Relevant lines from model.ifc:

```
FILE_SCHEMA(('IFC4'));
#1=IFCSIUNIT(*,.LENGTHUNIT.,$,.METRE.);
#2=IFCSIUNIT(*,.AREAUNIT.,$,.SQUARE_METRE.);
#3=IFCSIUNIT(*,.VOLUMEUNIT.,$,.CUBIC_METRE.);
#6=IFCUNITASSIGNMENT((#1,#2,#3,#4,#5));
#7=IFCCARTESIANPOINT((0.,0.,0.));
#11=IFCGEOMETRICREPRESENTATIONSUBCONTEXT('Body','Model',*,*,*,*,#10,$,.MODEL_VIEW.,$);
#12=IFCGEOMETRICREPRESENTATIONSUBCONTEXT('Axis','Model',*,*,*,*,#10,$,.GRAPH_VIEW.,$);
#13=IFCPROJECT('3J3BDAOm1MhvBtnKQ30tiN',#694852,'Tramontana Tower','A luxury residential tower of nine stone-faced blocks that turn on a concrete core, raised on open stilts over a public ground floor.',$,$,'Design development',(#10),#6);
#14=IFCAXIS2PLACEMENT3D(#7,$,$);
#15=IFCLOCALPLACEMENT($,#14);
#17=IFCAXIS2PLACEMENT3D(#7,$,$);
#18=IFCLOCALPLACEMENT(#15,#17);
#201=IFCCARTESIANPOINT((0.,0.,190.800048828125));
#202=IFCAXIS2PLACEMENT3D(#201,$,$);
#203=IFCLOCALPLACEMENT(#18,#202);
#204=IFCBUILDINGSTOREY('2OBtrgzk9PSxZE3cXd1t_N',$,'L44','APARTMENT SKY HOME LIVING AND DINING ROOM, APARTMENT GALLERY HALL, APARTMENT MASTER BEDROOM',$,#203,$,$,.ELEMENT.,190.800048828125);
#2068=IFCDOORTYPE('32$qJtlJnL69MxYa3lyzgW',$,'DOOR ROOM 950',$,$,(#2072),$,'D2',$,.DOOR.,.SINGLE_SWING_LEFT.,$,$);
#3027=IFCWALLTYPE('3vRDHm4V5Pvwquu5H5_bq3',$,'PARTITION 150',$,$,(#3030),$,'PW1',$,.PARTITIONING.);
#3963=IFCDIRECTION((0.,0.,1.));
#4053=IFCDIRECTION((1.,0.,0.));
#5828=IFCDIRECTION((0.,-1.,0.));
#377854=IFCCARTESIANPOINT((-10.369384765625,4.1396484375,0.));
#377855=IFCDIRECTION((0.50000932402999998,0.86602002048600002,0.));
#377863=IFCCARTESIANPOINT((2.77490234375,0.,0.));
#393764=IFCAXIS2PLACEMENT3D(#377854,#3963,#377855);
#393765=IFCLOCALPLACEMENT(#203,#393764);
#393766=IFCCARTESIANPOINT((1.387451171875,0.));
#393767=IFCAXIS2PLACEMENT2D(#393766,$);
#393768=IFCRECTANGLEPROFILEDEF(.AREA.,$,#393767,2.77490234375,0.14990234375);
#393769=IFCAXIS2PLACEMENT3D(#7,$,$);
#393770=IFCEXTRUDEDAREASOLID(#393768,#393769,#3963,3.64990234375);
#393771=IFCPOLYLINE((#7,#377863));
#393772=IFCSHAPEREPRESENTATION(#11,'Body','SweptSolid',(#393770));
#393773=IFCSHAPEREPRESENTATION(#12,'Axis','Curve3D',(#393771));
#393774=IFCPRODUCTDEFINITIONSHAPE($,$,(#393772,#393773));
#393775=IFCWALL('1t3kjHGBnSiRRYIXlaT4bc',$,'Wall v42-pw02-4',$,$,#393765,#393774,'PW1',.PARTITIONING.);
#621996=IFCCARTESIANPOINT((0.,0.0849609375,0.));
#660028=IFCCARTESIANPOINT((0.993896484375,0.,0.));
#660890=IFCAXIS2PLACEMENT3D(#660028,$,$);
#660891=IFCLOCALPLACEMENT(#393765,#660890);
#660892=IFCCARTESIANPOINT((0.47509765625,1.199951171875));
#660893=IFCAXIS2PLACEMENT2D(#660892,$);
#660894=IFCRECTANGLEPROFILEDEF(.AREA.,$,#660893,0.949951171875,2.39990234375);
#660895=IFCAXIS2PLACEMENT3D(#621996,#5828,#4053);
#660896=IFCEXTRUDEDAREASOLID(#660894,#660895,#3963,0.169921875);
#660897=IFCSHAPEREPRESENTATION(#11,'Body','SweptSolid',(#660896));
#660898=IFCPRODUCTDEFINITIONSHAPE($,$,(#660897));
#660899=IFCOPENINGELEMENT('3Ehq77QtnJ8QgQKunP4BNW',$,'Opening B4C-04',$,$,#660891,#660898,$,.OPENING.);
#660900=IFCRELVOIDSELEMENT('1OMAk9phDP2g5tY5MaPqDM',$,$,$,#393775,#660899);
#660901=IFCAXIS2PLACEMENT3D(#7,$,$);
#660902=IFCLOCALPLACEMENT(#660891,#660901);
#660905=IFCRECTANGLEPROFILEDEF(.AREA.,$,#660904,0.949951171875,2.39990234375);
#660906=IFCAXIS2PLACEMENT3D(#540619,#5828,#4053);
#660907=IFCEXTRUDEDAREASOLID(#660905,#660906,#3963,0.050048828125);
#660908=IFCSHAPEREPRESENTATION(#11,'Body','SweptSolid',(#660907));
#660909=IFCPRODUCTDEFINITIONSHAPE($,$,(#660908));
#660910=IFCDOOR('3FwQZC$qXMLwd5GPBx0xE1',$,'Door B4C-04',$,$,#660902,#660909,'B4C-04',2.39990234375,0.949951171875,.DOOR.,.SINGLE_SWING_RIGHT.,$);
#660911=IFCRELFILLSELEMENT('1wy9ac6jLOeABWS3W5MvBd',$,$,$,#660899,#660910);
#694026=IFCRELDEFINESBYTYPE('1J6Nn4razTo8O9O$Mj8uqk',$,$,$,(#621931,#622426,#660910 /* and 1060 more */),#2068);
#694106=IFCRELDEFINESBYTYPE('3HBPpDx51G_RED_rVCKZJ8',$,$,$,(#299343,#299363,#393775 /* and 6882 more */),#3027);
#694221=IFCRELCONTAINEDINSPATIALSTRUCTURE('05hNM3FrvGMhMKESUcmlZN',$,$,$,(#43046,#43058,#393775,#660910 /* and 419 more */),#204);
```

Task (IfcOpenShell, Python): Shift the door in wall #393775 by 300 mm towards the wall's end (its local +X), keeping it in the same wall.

```python
import ifcopenshell
import ifcopenshell.api.geometry
import ifcopenshell.util.placement
import ifcopenshell.util.unit

model = ifcopenshell.open("model.ifc")
unit_scale = ifcopenshell.util.unit.calculate_unit_scale(model)

door = model.by_guid("3FwQZC$qXMLwd5GPBx0xE1")
opening = door.FillsVoids[0].RelatingOpeningElement
wall = opening.VoidsElements[0].RelatingBuildingElement

wall_matrix = ifcopenshell.util.placement.get_local_placement(wall.ObjectPlacement)
shift = wall_matrix[:3, 0] * 0.3 / unit_scale
before = ifcopenshell.util.placement.get_local_placement(door.ObjectPlacement)[:3, 3].copy()

# The door is placed relative to its opening, so it follows when the opening moves.
matrix = ifcopenshell.util.placement.get_local_placement(opening.ObjectPlacement)
matrix[:3, 3] += shift
ifcopenshell.api.geometry.edit_object_placement(
    model, product=opening, matrix=matrix, is_si=False, should_transform_children=True
)

after = ifcopenshell.util.placement.get_local_placement(door.ObjectPlacement)[:3, 3]
print("door moved by", (after - before).round(3) + 0.0)

model.write("model-out.ifc")
```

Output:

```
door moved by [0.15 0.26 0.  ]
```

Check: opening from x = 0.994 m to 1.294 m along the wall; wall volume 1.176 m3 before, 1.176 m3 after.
